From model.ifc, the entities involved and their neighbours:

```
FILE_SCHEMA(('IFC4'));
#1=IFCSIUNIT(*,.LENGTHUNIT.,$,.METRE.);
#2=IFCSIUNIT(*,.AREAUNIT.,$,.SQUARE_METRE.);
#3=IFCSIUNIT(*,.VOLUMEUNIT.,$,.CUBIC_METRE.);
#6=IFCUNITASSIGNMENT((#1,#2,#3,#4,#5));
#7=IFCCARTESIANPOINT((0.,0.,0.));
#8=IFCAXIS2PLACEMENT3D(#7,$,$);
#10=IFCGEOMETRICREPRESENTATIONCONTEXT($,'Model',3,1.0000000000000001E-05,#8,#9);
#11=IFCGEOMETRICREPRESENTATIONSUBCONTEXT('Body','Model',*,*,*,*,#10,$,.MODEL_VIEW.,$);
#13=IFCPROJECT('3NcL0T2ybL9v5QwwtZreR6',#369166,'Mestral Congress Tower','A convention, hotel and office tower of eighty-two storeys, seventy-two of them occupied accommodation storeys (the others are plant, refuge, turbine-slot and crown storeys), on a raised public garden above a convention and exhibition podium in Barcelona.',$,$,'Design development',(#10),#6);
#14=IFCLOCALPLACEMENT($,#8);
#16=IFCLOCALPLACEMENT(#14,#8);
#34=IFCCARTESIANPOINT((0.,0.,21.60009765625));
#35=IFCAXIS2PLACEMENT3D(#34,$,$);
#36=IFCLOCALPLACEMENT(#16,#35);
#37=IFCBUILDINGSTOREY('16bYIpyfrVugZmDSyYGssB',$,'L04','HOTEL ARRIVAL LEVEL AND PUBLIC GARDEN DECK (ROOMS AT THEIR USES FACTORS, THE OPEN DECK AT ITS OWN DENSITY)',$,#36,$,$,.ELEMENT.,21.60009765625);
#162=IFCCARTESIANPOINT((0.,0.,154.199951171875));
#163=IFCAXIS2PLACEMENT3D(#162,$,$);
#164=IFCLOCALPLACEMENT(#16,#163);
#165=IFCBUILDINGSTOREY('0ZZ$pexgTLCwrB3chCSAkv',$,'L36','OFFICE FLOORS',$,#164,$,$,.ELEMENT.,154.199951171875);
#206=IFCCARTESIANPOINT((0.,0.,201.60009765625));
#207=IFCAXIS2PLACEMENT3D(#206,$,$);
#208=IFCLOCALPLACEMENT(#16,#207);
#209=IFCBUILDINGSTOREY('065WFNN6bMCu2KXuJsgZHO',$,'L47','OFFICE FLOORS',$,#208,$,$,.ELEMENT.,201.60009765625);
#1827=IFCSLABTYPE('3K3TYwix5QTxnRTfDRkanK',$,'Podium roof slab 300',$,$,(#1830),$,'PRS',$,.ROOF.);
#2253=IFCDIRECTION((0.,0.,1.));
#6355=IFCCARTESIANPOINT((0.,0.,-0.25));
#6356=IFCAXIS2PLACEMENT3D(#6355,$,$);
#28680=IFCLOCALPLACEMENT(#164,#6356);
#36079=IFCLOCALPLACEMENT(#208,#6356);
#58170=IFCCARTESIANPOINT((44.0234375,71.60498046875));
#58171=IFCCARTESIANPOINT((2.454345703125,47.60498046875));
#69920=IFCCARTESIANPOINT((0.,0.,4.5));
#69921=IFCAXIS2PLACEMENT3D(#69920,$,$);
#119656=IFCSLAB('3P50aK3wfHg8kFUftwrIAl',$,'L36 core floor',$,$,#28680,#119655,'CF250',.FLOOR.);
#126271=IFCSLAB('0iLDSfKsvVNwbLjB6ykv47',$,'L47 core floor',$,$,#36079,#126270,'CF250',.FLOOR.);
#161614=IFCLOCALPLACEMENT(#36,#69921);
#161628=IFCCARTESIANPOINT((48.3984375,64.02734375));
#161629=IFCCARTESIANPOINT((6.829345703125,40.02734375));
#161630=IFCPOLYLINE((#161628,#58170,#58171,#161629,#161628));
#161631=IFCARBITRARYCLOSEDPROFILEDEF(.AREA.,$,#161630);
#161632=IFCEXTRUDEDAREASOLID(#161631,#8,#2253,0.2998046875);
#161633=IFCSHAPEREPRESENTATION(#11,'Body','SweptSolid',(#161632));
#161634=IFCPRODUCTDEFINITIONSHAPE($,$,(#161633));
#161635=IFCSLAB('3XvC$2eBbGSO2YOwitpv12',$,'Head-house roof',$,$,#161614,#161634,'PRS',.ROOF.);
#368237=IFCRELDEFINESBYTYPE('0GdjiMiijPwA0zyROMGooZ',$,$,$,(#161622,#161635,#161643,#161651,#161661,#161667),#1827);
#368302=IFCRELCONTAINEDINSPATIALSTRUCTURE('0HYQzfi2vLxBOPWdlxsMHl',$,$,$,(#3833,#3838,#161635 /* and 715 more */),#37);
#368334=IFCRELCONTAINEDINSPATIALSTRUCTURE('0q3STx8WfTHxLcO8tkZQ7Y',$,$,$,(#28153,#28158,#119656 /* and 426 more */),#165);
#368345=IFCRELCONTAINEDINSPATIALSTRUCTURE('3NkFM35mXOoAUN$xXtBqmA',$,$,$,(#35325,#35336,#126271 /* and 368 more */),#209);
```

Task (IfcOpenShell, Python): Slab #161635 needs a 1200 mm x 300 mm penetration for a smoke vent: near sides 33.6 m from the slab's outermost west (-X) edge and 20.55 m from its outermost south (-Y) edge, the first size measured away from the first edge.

```python
import numpy as np
import ifcopenshell
import ifcopenshell.api.feature
import ifcopenshell.api.geometry
import ifcopenshell.api.root
import ifcopenshell.geom
import ifcopenshell.util.placement
import ifcopenshell.util.representation
import ifcopenshell.util.shape
import ifcopenshell.util.unit

model = ifcopenshell.open("model.ifc")
unit_scale = ifcopenshell.util.unit.calculate_unit_scale(model)
settings = ifcopenshell.geom.settings()


def volume(element):
    """Net volume in cubic metres, openings subtracted."""
    shape = ifcopenshell.geom.create_shape(settings, element)
    return ifcopenshell.util.shape.get_volume(shape.geometry)


slab = model.by_guid("3XvC$2eBbGSO2YOwitpv12")
before = volume(slab)

# Extent in the slab's own axes, in metres. The edges named are its -X and -Y sides.
slab_shape = ifcopenshell.geom.create_shape(settings, slab)
vertices = ifcopenshell.util.shape.get_vertices(slab_shape.geometry)
x_min, y_min, bottom = vertices.min(axis=0)
top = vertices[:, 2].max()

opening = ifcopenshell.api.root.create_entity(model, ifc_class="IfcOpeningElement", name="Smoke vent opening", predefined_type="OPENING")
context = ifcopenshell.util.representation.get_context(model, "Model", "Body", "MODEL_VIEW")
width, depth = 1.2, 0.3
outline = [(0.0, 0.0), (width, 0.0), (width, depth), (0.0, depth), (0.0, 0.0)]
# Overshoot both faces by 50 mm so the cut is clean.
shape = ifcopenshell.api.geometry.add_slab_representation(
    model, context=context, depth=top - bottom + 0.1, polyline=outline
)
ifcopenshell.api.geometry.assign_representation(model, product=opening, representation=shape)

matrix = ifcopenshell.util.placement.get_local_placement(slab.ObjectPlacement)
matrix[:, 3] = matrix @ np.append(np.array([x_min + 33.6, y_min + 20.55, bottom - 0.05]) / unit_scale, 1.0)
ifcopenshell.api.geometry.edit_object_placement(model, product=opening, matrix=matrix, is_si=False)
ifcopenshell.api.feature.add_feature(model, feature=opening, element=slab)

after = volume(slab)

print(f"slab volume {before:.3f} -> {after:.3f} m3")

model.write("model_v2.ifc")
```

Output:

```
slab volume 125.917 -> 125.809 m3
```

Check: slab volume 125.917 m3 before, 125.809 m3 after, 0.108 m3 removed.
